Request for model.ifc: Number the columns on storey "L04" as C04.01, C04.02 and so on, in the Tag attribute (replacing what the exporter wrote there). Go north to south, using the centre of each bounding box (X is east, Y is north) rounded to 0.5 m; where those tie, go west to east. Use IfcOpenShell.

First a look at what the model holds.

```python
import ifcopenshell
import ifcopenshell.util.element
import ifcopenshell.util.placement

model = ifcopenshell.open("model.ifc")
print(model.schema)
storey = next(s for s in model.by_type("IfcBuildingStorey") if s.Name == "L04")
columns = [e for e in ifcopenshell.util.element.get_decomposition(storey) if e.is_a("IfcColumn")]
for e in sorted(columns, key=lambda e: e.id()):
    origin = ifcopenshell.util.placement.get_local_placement(e.ObjectPlacement)[:3, 3]
    print(e.id(), e.Tag, e.Name, origin.round(2) + 0.0, sep=" | ")
```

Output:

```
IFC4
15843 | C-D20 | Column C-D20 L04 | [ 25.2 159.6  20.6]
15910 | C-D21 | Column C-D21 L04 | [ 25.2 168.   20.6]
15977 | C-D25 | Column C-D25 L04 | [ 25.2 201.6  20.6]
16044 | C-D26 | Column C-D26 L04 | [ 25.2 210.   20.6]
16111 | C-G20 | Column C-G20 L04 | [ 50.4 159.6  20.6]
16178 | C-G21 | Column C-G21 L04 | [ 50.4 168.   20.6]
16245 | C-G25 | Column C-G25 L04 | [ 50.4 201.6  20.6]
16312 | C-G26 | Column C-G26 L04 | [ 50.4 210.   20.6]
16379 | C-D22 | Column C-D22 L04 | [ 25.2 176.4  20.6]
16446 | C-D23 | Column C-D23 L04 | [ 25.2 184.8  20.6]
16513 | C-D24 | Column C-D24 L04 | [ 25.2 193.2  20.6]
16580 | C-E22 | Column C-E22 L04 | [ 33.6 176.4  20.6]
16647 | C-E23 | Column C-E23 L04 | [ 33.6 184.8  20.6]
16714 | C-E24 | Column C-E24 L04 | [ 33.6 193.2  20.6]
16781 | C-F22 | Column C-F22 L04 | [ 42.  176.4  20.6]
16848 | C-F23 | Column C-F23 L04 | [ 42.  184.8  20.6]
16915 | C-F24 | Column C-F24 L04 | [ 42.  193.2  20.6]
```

```python
import ifcopenshell
import ifcopenshell.geom
import ifcopenshell.util.element
import ifcopenshell.util.shape

model = ifcopenshell.open("model.ifc")
settings = ifcopenshell.geom.settings()
settings.set("use-world-coords", True)


def centre(element):
    shape = ifcopenshell.geom.create_shape(settings, element)
    return ifcopenshell.util.shape.get_bbox_centroid(shape.geometry)


storey = next(s for s in model.by_type("IfcBuildingStorey") if s.Name == "L04")
columns = [e for e in ifcopenshell.util.element.get_decomposition(storey) if e.is_a("IfcColumn")]

# Insertion points can sit at a corner or the storey origin, so sort by the geometry (in metres).
centres = {e: centre(e) for e in columns}
columns.sort(key=lambda e: (-round(centres[e][1] / 0.5), centres[e][0]))

for i, e in enumerate(columns, start=1):
    number = f"C04.{i:02d}"
    e.Tag = number
    print(e.id(), number)

model.write("model-out.ifc")
```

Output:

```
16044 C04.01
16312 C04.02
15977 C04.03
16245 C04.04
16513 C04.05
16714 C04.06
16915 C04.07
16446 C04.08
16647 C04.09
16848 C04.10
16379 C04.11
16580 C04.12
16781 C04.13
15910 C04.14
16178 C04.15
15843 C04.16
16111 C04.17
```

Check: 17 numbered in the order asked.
